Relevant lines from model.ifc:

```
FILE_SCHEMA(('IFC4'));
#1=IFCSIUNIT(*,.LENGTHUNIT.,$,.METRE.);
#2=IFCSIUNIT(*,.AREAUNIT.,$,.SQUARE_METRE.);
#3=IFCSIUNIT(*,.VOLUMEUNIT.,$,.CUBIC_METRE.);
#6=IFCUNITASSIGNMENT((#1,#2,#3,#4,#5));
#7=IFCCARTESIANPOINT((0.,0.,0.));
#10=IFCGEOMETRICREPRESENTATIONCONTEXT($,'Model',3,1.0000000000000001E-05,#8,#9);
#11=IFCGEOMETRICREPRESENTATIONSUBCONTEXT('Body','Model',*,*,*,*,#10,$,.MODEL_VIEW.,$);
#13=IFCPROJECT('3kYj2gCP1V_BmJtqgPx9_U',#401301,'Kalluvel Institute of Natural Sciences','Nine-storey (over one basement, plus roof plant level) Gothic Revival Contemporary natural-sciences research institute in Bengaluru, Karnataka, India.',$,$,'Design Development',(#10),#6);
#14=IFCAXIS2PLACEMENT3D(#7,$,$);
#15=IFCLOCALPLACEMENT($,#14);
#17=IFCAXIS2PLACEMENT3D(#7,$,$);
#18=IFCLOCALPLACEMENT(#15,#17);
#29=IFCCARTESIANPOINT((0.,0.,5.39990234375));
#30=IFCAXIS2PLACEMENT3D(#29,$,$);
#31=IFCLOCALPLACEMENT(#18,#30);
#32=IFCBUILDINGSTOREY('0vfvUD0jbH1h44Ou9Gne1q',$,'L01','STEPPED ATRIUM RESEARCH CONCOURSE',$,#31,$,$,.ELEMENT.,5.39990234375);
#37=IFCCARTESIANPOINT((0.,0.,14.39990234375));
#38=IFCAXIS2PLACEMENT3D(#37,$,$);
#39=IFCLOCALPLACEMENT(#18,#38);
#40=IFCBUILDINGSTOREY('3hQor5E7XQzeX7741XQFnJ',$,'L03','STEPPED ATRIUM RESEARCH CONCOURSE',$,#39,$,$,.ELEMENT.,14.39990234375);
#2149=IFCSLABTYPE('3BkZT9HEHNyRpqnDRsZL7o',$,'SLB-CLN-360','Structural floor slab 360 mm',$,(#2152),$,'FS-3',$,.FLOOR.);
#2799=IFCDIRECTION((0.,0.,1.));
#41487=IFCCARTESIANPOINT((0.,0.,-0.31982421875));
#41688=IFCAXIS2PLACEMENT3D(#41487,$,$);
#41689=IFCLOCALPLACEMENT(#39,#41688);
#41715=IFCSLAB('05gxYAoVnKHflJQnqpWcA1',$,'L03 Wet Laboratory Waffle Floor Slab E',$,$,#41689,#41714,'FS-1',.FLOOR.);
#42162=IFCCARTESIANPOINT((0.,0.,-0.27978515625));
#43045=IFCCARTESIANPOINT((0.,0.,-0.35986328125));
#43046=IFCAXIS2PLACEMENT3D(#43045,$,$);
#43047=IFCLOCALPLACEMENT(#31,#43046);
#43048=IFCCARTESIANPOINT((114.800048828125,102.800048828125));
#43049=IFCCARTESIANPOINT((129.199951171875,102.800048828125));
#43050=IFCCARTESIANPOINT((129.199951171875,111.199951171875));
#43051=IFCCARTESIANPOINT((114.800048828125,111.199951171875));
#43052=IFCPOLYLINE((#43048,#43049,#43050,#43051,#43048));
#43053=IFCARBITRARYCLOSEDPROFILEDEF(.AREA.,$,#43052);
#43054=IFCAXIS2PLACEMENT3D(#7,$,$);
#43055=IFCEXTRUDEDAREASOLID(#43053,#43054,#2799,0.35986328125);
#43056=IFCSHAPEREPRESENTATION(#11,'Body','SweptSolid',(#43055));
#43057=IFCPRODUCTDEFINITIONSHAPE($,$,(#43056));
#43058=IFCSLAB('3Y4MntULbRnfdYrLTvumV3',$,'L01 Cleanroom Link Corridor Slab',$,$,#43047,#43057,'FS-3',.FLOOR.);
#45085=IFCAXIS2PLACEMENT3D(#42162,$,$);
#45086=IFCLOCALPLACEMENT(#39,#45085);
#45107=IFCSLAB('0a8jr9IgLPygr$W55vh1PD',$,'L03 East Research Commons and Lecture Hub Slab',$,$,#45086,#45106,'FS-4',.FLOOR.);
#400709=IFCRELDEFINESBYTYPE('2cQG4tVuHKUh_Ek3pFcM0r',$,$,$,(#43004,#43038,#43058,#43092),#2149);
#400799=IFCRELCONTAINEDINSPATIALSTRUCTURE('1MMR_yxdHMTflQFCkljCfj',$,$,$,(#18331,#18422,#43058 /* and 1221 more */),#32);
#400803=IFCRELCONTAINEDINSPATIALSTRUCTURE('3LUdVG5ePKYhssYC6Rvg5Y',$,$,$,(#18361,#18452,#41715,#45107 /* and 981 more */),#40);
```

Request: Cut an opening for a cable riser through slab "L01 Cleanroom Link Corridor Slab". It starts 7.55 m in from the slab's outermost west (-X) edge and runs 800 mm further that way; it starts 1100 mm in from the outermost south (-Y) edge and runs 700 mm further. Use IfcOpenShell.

```python
import numpy as np
import ifcopenshell
import ifcopenshell.api.feature
import ifcopenshell.api.geometry
import ifcopenshell.api.root
import ifcopenshell.geom
import ifcopenshell.util.placement
import ifcopenshell.util.representation
import ifcopenshell.util.shape
import ifcopenshell.util.unit

model = ifcopenshell.open("model.ifc")
unit_scale = ifcopenshell.util.unit.calculate_unit_scale(model)
settings = ifcopenshell.geom.settings()


def volume(element):
    """Net volume in cubic metres, openings subtracted."""
    shape = ifcopenshell.geom.create_shape(settings, element)
    return ifcopenshell.util.shape.get_volume(shape.geometry)


slab = model.by_guid("3Y4MntULbRnfdYrLTvumV3")
before = volume(slab)

# Extent in the slab's own axes, in metres. The edges named are its -X and -Y sides.
slab_shape = ifcopenshell.geom.create_shape(settings, slab)
vertices = ifcopenshell.util.shape.get_vertices(slab_shape.geometry)
x_min, y_min, bottom = vertices.min(axis=0)
top = vertices[:, 2].max()

opening = ifcopenshell.api.root.create_entity(model, ifc_class="IfcOpeningElement", name="Cable riser opening", predefined_type="OPENING")
context = ifcopenshell.util.representation.get_context(model, "Model", "Body", "MODEL_VIEW")
width, depth = 0.8, 0.7
outline = [(0.0, 0.0), (width, 0.0), (width, depth), (0.0, depth), (0.0, 0.0)]
# Overshoot both faces by 50 mm so the cut is clean.
shape = ifcopenshell.api.geometry.add_slab_representation(
    model, context=context, depth=top - bottom + 0.1, polyline=outline
)
ifcopenshell.api.geometry.assign_representation(model, product=opening, representation=shape)

matrix = ifcopenshell.util.placement.get_local_placement(slab.ObjectPlacement)
matrix[:, 3] = matrix @ np.append(np.array([x_min + 7.55, y_min + 1.1, bottom - 0.05]) / unit_scale, 1.0)
ifcopenshell.api.geometry.edit_object_placement(model, product=opening, matrix=matrix, is_si=False)
ifcopenshell.api.feature.add_feature(model, feature=opening, element=slab)

after = volume(slab)

print(f"slab volume {before:.3f} -> {after:.3f} m3")

model.write("model_v2.ifc")
```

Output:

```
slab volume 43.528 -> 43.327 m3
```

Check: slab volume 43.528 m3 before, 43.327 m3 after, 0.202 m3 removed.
